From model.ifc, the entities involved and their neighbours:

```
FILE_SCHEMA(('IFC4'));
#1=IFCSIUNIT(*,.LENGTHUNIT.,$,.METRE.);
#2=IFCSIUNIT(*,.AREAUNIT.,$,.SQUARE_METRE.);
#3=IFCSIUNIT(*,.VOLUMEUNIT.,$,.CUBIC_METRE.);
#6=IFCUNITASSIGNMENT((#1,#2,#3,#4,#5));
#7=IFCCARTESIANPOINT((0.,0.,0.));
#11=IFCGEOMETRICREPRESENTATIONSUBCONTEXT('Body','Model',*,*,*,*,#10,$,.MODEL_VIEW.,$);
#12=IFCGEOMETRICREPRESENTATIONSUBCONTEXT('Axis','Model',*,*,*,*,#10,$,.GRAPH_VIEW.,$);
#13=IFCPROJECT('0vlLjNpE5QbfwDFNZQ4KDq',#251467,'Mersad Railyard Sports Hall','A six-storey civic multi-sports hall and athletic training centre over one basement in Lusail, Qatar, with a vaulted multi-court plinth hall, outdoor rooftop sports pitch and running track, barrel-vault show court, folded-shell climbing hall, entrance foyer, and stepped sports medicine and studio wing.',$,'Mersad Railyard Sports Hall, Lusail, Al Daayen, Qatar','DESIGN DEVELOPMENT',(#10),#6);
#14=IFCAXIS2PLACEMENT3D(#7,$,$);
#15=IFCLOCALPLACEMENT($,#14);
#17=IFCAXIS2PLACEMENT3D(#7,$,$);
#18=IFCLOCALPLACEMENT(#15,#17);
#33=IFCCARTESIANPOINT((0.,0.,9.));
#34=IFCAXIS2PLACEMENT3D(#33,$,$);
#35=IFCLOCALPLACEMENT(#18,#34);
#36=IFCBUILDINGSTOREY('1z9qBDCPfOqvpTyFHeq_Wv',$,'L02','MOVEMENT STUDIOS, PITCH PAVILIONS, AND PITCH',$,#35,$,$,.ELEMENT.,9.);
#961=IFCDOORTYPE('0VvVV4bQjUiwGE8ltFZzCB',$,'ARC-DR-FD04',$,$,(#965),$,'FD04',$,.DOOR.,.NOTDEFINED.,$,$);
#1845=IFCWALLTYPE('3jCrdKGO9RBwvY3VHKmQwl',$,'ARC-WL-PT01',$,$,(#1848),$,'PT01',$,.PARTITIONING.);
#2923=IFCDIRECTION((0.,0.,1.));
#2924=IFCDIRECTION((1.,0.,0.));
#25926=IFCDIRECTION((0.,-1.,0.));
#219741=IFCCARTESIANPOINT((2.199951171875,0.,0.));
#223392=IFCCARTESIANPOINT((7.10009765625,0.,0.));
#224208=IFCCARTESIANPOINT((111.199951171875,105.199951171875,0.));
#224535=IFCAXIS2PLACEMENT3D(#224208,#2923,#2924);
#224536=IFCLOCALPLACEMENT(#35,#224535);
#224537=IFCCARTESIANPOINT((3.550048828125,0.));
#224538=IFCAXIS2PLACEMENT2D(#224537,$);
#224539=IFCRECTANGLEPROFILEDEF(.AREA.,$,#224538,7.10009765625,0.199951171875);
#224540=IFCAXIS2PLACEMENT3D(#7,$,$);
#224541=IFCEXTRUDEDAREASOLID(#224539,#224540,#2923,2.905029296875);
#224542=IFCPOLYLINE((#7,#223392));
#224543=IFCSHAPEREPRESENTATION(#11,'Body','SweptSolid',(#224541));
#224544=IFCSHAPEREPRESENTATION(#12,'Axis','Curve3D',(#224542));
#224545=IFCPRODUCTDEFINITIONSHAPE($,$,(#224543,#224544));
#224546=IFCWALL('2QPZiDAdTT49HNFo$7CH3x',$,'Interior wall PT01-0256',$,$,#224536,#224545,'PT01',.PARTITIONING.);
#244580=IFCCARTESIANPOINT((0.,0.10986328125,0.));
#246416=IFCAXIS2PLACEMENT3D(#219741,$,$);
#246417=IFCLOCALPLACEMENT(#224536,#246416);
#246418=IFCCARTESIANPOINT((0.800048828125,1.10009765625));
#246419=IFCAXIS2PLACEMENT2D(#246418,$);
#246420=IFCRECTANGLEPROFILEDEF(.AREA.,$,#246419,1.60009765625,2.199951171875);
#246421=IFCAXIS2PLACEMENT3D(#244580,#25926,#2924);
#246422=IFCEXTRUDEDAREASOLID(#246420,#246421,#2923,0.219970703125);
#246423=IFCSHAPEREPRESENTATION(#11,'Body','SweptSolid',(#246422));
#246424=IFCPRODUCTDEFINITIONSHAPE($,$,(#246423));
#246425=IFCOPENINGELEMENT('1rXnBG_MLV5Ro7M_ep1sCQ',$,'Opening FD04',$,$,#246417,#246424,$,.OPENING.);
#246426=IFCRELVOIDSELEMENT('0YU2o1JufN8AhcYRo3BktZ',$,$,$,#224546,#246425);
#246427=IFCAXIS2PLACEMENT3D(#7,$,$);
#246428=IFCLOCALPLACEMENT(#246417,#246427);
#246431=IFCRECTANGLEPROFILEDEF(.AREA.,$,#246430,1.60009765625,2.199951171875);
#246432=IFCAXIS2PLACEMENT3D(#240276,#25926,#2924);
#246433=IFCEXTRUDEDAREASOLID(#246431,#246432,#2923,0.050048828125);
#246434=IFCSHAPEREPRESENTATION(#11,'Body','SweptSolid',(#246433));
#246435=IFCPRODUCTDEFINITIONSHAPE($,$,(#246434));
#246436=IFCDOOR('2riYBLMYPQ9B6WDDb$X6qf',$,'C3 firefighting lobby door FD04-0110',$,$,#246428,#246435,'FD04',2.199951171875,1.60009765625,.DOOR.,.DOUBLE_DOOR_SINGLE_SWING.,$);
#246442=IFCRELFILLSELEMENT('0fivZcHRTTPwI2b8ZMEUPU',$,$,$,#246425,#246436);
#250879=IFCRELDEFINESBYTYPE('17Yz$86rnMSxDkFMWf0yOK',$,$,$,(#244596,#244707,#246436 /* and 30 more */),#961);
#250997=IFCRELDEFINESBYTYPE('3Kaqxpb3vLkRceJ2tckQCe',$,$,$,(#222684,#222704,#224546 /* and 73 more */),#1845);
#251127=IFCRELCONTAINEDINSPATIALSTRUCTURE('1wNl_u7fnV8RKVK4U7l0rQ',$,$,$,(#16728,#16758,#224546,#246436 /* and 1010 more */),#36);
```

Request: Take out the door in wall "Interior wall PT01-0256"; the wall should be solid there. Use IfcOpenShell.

```python
import ifcopenshell
import ifcopenshell.api.feature
import ifcopenshell.api.root
import ifcopenshell.geom
import ifcopenshell.util.shape

model = ifcopenshell.open("model.ifc")
settings = ifcopenshell.geom.settings()


def volume(element):
    """Net volume in cubic metres, openings subtracted."""
    shape = ifcopenshell.geom.create_shape(settings, element)
    return ifcopenshell.util.shape.get_volume(shape.geometry)


door = model.by_guid("2riYBLMYPQ9B6WDDb$X6qf")
opening = door.FillsVoids[0].RelatingOpeningElement
wall = opening.VoidsElements[0].RelatingBuildingElement
before = volume(wall)

ifcopenshell.api.root.remove_product(model, product=door)
ifcopenshell.api.feature.remove_feature(model, feature=opening)

after = volume(wall)

print(f"wall volume {before:.3f} -> {after:.3f} m3")

model.write("model-out.ifc")
```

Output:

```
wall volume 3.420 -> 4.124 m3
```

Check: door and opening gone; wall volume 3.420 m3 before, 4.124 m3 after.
